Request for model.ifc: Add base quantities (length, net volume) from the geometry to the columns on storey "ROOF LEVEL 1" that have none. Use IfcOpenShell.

First a look at what the model holds.

```python
import ifcopenshell
import ifcopenshell.util.element
import ifcopenshell.util.unit

model = ifcopenshell.open("model.ifc")
print(model.schema)
for unit_type in ("LENGTHUNIT", "AREAUNIT", "VOLUMEUNIT"):
    print(unit_type, ifcopenshell.util.unit.calculate_unit_scale(model, unit_type))
storey = next(s for s in model.by_type("IfcBuildingStorey") if s.Name == "ROOF LEVEL 1")
columns = [e for e in ifcopenshell.util.element.get_decomposition(storey) if e.is_a("IfcColumn")]
for e in sorted(columns, key=lambda e: e.id()):
    print(e.id(), e.is_a(), e.Name, list(ifcopenshell.util.element.get_psets(e, qtos_only=True)), sep=" | ")
```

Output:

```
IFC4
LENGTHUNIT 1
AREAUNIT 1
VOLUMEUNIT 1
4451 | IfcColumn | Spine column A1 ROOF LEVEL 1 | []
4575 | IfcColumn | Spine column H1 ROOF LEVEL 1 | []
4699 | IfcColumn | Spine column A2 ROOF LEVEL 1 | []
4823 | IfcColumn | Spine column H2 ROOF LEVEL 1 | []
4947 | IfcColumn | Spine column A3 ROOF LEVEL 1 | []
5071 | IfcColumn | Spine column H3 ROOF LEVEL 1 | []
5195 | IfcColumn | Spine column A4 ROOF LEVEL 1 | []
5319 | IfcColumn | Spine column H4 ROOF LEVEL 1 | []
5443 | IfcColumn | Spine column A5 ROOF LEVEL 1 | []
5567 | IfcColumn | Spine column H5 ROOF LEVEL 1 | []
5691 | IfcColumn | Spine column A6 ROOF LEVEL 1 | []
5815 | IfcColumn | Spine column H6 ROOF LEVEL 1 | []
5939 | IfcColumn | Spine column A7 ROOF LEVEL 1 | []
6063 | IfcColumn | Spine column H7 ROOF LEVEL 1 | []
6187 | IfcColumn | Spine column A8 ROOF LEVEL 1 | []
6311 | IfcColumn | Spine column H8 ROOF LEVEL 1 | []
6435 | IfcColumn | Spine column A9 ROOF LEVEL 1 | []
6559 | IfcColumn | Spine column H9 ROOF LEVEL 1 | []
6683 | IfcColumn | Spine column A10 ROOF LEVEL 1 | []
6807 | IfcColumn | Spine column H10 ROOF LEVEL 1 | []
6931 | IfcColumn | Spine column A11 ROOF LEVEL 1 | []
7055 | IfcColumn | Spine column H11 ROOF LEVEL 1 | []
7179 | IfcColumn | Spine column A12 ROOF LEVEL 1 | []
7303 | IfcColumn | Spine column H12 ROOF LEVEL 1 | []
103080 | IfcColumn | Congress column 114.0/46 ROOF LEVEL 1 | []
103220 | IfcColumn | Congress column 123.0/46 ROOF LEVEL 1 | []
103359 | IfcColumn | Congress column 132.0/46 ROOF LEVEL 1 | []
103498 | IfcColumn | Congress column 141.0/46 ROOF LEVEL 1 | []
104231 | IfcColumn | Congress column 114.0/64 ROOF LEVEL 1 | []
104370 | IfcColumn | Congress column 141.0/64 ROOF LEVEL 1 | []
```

```python
import ifcopenshell
import ifcopenshell.api.pset
import ifcopenshell.geom
import ifcopenshell.util.element
import ifcopenshell.util.shape
import ifcopenshell.util.unit

model = ifcopenshell.open("model.ifc")
unit_scale = ifcopenshell.util.unit.calculate_unit_scale(model)
volume_scale = ifcopenshell.util.unit.calculate_unit_scale(model, "VOLUMEUNIT")
settings = ifcopenshell.geom.settings()

storey = next(s for s in model.by_type("IfcBuildingStorey") if s.Name == "ROOF LEVEL 1")
columns = [e for e in ifcopenshell.util.element.get_decomposition(storey) if e.is_a("IfcColumn")]

for e in sorted(columns, key=lambda e: e.id()):
    if ifcopenshell.util.element.get_psets(e, qtos_only=True, should_inherit=False):
        continue
    # Geometry comes back in metres, in the element's own axes.
    shape = ifcopenshell.geom.create_shape(settings, e)
    values = {
        "Length": ifcopenshell.util.shape.get_z(shape.geometry) / unit_scale,
        "NetVolume": ifcopenshell.util.shape.get_volume(shape.geometry) / volume_scale,
    }
    qto = ifcopenshell.api.pset.add_qto(model, product=e, name="Qto_ColumnBaseQuantities")
    ifcopenshell.api.pset.edit_qto(model, qto=qto, properties=values)
    print(e.id(), {k: round(v, 3) for k, v in values.items()})

model.write("model_v2.ifc")
```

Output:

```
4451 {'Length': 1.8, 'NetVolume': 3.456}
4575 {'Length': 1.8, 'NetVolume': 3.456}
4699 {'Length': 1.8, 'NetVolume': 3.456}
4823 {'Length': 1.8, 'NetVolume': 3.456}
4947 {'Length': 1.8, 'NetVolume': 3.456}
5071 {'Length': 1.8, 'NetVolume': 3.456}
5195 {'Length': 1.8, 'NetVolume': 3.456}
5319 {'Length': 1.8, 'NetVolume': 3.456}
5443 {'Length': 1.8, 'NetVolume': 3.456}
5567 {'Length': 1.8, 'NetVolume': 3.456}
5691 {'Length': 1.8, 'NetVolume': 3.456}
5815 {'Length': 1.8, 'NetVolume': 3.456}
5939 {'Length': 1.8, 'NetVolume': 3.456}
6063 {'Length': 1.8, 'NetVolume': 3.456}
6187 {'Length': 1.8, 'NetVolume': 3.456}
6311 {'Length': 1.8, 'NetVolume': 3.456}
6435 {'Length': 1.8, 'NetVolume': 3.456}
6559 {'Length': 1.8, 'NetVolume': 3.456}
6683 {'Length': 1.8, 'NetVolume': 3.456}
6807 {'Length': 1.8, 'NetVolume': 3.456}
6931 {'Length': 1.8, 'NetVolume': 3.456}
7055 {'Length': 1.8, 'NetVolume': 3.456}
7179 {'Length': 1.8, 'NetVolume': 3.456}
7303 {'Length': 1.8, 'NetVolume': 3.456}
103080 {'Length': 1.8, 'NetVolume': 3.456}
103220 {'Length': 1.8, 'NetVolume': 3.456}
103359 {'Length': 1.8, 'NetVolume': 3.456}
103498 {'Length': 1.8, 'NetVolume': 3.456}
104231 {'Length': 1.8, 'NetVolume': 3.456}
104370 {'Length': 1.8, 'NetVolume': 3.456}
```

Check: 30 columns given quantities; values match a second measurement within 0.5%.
